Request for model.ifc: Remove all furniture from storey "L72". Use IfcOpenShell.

First a look at what the model holds.

```python
import ifcopenshell
import ifcopenshell.util.element

model = ifcopenshell.open("model.ifc")
print(model.schema)
storey = next(s for s in model.by_type("IfcBuildingStorey") if s.Name == "L72")
furniture = [e for e in ifcopenshell.util.element.get_decomposition(storey) if e.is_a("IfcFurnishingElement")]
seen = {}
for e in furniture:
    element_type = ifcopenshell.util.element.get_type(e)
    name = element_type.Name if element_type not in (None, e) else None
    seen[name] = seen.get(name, 0) + 1
for name, count in sorted(seen.items(), key=str):
    print(count, "x", name)
```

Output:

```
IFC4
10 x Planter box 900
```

```python
import ifcopenshell
import ifcopenshell.api.root
import ifcopenshell.util.element

model = ifcopenshell.open("model.ifc")

storey = next(s for s in model.by_type("IfcBuildingStorey") if s.Name == "L72")
furniture = [e for e in ifcopenshell.util.element.get_decomposition(storey) if e.is_a("IfcFurnishingElement")]

for e in furniture:
    ifcopenshell.api.root.remove_product(model, product=e)
print(len(furniture), "removed")

model.write("model_rev.ifc")
```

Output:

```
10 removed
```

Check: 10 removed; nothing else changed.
